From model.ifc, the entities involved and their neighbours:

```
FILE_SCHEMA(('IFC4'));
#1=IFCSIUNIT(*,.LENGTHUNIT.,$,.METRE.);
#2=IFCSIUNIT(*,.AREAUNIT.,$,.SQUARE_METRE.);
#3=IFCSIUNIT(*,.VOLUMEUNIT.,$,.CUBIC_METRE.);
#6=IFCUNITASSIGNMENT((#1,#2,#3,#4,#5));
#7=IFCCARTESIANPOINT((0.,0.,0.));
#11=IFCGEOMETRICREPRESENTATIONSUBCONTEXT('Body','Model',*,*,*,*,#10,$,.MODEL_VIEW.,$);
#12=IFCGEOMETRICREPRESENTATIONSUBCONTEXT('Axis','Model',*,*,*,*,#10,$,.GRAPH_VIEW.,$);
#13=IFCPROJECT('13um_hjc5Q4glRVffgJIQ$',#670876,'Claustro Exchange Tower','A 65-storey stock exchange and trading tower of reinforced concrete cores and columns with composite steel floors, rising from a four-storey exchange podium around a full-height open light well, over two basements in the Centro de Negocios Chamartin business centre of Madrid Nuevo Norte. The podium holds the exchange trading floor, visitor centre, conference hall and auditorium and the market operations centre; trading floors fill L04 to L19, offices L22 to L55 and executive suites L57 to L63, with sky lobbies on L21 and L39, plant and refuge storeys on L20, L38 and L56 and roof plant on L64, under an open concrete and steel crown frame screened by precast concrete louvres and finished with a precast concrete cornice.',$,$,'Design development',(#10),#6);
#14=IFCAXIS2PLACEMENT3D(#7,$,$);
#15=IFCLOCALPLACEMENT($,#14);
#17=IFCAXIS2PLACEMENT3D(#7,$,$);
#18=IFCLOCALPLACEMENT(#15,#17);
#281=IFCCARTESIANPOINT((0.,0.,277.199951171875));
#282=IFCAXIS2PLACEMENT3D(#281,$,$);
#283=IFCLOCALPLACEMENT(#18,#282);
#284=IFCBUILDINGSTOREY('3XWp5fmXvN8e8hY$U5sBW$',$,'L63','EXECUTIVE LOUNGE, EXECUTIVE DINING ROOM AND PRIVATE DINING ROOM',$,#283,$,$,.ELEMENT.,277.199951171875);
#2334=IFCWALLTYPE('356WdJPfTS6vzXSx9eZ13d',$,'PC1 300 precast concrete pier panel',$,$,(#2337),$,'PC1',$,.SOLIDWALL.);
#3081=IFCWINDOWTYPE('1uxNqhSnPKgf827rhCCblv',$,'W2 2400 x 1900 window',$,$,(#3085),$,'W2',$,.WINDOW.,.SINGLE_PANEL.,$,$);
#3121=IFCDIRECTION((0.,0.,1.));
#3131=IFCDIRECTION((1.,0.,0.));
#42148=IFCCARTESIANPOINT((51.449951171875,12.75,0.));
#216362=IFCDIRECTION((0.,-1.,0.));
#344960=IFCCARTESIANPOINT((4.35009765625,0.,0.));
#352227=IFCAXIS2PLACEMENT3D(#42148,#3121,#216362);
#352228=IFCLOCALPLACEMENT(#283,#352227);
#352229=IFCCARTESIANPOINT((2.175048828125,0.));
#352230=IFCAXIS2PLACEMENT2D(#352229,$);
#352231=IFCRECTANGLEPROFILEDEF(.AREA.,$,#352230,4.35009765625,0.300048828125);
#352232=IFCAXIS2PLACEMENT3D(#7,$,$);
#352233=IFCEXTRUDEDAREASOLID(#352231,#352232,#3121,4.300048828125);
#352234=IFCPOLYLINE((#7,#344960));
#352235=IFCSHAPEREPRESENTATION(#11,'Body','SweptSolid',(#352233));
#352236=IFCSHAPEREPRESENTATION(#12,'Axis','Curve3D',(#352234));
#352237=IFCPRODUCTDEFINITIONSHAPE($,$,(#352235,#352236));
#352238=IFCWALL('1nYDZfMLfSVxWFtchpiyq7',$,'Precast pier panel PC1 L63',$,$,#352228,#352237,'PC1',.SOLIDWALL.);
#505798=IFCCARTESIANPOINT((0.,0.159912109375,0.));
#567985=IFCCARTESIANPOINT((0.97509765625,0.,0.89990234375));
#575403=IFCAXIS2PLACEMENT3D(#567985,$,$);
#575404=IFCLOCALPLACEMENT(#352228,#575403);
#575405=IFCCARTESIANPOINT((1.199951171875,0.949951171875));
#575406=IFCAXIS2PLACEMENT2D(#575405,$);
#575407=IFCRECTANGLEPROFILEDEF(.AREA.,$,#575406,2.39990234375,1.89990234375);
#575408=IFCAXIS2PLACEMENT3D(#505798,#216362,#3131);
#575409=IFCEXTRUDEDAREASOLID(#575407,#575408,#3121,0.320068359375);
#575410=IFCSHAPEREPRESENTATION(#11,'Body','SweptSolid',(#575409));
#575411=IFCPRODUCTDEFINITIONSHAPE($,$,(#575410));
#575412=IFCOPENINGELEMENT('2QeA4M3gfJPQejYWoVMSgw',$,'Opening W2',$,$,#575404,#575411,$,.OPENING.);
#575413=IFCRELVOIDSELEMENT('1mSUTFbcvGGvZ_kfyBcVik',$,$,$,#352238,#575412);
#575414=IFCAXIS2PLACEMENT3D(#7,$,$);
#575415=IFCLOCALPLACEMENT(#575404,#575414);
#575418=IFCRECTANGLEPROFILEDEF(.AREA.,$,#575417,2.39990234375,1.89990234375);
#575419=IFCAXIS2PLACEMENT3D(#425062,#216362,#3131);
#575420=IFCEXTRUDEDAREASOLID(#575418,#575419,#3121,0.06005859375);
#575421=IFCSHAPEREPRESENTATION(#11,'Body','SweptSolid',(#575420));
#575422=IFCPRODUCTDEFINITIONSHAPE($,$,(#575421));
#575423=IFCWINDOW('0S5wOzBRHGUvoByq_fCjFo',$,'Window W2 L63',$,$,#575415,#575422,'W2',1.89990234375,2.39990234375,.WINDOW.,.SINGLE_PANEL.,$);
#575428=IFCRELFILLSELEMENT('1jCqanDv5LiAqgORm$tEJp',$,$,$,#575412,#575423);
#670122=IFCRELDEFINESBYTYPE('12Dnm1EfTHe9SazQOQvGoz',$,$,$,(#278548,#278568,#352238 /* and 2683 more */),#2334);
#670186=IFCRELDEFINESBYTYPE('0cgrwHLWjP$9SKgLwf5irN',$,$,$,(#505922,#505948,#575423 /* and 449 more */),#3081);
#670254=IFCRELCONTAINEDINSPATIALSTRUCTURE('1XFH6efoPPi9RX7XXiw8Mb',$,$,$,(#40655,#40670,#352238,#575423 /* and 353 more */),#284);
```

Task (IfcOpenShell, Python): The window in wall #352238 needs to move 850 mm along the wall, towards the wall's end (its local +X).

```python
import ifcopenshell
import ifcopenshell.api.geometry
import ifcopenshell.util.placement
import ifcopenshell.util.unit

model = ifcopenshell.open("model.ifc")
unit_scale = ifcopenshell.util.unit.calculate_unit_scale(model)

window = model.by_guid("0S5wOzBRHGUvoByq_fCjFo")
opening = window.FillsVoids[0].RelatingOpeningElement
wall = opening.VoidsElements[0].RelatingBuildingElement

wall_matrix = ifcopenshell.util.placement.get_local_placement(wall.ObjectPlacement)
shift = wall_matrix[:3, 0] * 0.85 / unit_scale
before = ifcopenshell.util.placement.get_local_placement(window.ObjectPlacement)[:3, 3].copy()

# The window is placed relative to its opening, so it follows when the opening moves.
matrix = ifcopenshell.util.placement.get_local_placement(opening.ObjectPlacement)
matrix[:3, 3] += shift
ifcopenshell.api.geometry.edit_object_placement(
    model, product=opening, matrix=matrix, is_si=False, should_transform_children=True
)

after = ifcopenshell.util.placement.get_local_placement(window.ObjectPlacement)[:3, 3]
print("window moved by", (after - before).round(3) + 0.0)

model.write("model_updated.ifc")
```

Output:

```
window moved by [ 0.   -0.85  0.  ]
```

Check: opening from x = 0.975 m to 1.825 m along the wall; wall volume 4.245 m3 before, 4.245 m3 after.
